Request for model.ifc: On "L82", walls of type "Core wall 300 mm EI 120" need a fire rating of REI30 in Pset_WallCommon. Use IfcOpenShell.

First a look at what the model holds.

```python
import ifcopenshell
import ifcopenshell.util.element

model = ifcopenshell.open("model.ifc")
print(model.schema)
storey = next(s for s in model.by_type("IfcBuildingStorey") if s.Name == "L82")
walls = [e for e in ifcopenshell.util.element.get_decomposition(storey) if e.is_a("IfcWall")]
seen = {}
for e in walls:
    element_type = ifcopenshell.util.element.get_type(e)
    key = (element_type.Name if element_type != e and element_type else None, ifcopenshell.util.element.get_pset(e, "Pset_WallCommon", "FireRating"))
    seen[key] = seen.get(key, 0) + 1
for (name, value), count in sorted(seen.items(), key=str):
    print(count, "x", name, "|", value)
```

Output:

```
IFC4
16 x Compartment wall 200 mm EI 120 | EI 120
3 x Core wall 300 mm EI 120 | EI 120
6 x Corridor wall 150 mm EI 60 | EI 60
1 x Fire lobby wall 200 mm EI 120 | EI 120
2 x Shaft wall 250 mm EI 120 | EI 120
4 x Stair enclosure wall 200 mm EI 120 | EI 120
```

```python
import ifcopenshell
import ifcopenshell.api.pset
import ifcopenshell.util.element

model = ifcopenshell.open("model.ifc")

storey = next(s for s in model.by_type("IfcBuildingStorey") if s.Name == "L82")
walls = [e for e in ifcopenshell.util.element.get_decomposition(storey) if e.is_a("IfcWall")]

count = 0
for e in walls:
    element_type = ifcopenshell.util.element.get_type(e)
    if element_type in (None, e) or element_type.Name != "Core wall 300 mm EI 120":
        continue
    found = ifcopenshell.util.element.get_pset(e, "Pset_WallCommon", should_inherit=False)
    if found:
        pset = model.by_id(found["id"])
        if len(ifcopenshell.util.element.get_elements_by_pset(pset)) > 1:
            pset = ifcopenshell.api.pset.unshare_pset(model, products=[e], pset=pset)[0]
    else:
        pset = ifcopenshell.api.pset.add_pset(model, product=e, name="Pset_WallCommon")
    ifcopenshell.api.pset.edit_pset(model, pset=pset, properties={"FireRating": "REI30"})
    count += 1

print(count, "walls updated")

model.write("model_rev.ifc")
```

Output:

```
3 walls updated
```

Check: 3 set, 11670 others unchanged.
